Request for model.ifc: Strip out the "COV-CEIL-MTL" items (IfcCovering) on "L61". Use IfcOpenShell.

First a look at what the model holds.

```python
import ifcopenshell
import ifcopenshell.util.element

model = ifcopenshell.open("model.ifc")
print(model.schema)
storey = next(s for s in model.by_type("IfcBuildingStorey") if s.Name == "L61")
coverings = [e for e in ifcopenshell.util.element.get_decomposition(storey) if e.is_a("IfcCovering")]
seen = {}
for e in coverings:
    element_type = ifcopenshell.util.element.get_type(e)
    name = element_type.Name if element_type not in (None, e) else None
    seen[name] = seen.get(name, 0) + 1
for name, count in sorted(seen.items(), key=str):
    print(count, "x", name)
```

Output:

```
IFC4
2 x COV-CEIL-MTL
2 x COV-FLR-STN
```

```python
import ifcopenshell
import ifcopenshell.api.root
import ifcopenshell.util.element

model = ifcopenshell.open("model.ifc")

storey = next(s for s in model.by_type("IfcBuildingStorey") if s.Name == "L61")
coverings = [e for e in ifcopenshell.util.element.get_decomposition(storey) if e.is_a("IfcCovering")]
targets = [e for e in coverings if (t := ifcopenshell.util.element.get_type(e)) not in (None, e) and t.Name == "COV-CEIL-MTL"]

for e in targets:
    ifcopenshell.api.root.remove_product(model, product=e)
print(len(targets), "removed")

model.write("model_edited.ifc")
```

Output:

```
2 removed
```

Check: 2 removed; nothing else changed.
